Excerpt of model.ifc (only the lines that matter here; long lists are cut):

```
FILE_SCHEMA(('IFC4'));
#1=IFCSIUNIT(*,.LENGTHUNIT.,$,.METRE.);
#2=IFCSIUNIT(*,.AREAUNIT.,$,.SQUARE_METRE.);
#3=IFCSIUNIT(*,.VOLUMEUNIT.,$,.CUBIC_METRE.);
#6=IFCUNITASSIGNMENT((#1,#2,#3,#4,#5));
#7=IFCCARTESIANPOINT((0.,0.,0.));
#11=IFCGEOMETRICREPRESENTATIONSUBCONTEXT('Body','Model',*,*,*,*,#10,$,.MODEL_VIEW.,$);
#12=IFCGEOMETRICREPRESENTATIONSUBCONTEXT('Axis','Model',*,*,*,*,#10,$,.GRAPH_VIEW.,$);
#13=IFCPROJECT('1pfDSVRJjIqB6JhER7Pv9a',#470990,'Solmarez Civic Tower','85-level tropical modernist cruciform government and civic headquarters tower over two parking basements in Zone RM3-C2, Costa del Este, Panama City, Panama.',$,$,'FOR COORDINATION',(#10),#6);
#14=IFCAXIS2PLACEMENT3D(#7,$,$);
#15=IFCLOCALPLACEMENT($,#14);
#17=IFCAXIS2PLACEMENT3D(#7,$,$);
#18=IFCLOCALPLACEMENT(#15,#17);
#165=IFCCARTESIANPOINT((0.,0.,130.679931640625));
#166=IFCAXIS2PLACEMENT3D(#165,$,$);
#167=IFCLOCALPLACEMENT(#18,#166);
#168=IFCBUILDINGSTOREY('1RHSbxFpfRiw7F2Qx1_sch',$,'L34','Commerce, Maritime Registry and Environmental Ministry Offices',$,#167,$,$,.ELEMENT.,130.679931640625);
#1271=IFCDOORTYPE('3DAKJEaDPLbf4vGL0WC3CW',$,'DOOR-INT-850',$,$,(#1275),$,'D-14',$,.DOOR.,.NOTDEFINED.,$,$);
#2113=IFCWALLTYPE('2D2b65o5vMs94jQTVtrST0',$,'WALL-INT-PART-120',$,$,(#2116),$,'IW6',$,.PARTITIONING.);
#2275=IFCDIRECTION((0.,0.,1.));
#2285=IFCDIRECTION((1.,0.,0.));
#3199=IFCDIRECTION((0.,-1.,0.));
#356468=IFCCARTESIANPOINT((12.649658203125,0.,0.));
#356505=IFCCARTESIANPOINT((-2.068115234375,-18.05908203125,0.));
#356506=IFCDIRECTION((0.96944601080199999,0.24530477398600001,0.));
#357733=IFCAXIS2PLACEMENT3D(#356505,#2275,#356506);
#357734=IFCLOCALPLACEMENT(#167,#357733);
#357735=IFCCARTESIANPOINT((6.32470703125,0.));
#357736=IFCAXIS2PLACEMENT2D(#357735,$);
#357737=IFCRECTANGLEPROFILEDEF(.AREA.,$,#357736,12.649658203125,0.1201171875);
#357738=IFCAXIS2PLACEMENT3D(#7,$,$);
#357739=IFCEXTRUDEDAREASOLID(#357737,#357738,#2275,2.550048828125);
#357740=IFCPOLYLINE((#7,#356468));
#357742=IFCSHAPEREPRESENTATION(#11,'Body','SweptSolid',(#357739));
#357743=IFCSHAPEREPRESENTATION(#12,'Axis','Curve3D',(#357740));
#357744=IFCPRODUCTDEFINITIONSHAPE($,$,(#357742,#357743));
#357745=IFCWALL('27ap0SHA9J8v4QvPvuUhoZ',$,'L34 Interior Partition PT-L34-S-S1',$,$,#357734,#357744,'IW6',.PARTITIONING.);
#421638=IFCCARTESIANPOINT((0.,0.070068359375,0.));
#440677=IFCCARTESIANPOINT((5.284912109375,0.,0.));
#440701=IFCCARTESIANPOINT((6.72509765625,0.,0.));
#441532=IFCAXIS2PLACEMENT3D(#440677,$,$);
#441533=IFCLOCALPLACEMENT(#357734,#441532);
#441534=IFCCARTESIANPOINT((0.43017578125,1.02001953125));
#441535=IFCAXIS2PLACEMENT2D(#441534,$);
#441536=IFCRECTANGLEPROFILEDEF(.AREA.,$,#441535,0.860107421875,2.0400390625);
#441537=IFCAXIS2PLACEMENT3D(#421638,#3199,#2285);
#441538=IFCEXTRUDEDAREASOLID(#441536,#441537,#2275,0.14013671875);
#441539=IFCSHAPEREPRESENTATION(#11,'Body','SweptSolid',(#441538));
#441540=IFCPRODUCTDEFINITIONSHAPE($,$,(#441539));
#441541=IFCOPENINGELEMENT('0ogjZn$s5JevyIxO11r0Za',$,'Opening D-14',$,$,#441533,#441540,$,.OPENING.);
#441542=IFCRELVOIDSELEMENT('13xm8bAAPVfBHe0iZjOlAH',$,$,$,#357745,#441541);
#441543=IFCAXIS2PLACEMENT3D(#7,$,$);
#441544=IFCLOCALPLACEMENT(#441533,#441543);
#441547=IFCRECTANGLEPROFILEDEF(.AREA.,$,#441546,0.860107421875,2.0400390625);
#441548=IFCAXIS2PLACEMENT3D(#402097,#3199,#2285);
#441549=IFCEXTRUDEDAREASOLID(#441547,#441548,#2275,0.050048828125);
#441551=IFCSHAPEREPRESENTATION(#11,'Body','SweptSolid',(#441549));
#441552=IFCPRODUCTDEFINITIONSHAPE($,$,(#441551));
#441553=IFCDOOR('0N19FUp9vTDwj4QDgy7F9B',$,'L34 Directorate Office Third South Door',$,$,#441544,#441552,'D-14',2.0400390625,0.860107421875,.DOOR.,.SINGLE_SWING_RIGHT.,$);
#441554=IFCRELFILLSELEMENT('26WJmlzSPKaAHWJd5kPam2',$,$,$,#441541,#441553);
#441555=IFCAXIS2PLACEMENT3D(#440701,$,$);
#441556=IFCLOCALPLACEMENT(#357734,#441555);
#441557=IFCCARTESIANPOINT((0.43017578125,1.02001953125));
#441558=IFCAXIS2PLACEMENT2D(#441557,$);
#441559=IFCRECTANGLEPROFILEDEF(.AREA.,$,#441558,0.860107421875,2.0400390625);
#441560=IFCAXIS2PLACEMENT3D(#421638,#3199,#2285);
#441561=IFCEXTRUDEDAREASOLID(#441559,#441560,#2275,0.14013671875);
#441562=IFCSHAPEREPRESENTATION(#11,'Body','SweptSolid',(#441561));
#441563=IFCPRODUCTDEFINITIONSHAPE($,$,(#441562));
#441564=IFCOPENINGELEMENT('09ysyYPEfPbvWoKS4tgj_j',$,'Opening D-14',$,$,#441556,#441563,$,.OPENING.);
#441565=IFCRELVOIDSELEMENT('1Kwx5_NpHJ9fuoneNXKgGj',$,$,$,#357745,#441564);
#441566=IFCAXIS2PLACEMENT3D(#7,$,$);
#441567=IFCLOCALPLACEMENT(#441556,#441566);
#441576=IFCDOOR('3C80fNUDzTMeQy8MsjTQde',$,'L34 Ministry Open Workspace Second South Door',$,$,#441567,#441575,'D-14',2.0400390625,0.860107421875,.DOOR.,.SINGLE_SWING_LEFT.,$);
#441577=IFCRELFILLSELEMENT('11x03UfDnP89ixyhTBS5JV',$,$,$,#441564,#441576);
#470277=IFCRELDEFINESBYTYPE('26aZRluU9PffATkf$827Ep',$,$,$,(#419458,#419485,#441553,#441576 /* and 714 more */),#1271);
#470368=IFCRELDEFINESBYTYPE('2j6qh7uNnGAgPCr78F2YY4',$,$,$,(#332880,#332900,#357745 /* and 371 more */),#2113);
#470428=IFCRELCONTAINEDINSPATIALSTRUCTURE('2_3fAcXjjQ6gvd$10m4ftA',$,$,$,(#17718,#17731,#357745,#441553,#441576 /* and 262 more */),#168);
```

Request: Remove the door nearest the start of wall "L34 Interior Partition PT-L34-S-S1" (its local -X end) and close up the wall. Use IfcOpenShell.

```python
import ifcopenshell
import ifcopenshell.api.feature
import ifcopenshell.api.root
import ifcopenshell.geom
import ifcopenshell.util.shape

model = ifcopenshell.open("model.ifc")
settings = ifcopenshell.geom.settings()


def volume(element):
    """Net volume in cubic metres, openings subtracted."""
    shape = ifcopenshell.geom.create_shape(settings, element)
    return ifcopenshell.util.shape.get_volume(shape.geometry)


door = model.by_guid("0N19FUp9vTDwj4QDgy7F9B")
opening = door.FillsVoids[0].RelatingOpeningElement
wall = opening.VoidsElements[0].RelatingBuildingElement
before = volume(wall)

ifcopenshell.api.root.remove_product(model, product=door)
ifcopenshell.api.feature.remove_feature(model, feature=opening)

after = volume(wall)

print(f"wall volume {before:.3f} -> {after:.3f} m3")

model.write("model-out.ifc")
```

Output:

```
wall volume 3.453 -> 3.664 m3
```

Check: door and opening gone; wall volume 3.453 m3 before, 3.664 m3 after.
